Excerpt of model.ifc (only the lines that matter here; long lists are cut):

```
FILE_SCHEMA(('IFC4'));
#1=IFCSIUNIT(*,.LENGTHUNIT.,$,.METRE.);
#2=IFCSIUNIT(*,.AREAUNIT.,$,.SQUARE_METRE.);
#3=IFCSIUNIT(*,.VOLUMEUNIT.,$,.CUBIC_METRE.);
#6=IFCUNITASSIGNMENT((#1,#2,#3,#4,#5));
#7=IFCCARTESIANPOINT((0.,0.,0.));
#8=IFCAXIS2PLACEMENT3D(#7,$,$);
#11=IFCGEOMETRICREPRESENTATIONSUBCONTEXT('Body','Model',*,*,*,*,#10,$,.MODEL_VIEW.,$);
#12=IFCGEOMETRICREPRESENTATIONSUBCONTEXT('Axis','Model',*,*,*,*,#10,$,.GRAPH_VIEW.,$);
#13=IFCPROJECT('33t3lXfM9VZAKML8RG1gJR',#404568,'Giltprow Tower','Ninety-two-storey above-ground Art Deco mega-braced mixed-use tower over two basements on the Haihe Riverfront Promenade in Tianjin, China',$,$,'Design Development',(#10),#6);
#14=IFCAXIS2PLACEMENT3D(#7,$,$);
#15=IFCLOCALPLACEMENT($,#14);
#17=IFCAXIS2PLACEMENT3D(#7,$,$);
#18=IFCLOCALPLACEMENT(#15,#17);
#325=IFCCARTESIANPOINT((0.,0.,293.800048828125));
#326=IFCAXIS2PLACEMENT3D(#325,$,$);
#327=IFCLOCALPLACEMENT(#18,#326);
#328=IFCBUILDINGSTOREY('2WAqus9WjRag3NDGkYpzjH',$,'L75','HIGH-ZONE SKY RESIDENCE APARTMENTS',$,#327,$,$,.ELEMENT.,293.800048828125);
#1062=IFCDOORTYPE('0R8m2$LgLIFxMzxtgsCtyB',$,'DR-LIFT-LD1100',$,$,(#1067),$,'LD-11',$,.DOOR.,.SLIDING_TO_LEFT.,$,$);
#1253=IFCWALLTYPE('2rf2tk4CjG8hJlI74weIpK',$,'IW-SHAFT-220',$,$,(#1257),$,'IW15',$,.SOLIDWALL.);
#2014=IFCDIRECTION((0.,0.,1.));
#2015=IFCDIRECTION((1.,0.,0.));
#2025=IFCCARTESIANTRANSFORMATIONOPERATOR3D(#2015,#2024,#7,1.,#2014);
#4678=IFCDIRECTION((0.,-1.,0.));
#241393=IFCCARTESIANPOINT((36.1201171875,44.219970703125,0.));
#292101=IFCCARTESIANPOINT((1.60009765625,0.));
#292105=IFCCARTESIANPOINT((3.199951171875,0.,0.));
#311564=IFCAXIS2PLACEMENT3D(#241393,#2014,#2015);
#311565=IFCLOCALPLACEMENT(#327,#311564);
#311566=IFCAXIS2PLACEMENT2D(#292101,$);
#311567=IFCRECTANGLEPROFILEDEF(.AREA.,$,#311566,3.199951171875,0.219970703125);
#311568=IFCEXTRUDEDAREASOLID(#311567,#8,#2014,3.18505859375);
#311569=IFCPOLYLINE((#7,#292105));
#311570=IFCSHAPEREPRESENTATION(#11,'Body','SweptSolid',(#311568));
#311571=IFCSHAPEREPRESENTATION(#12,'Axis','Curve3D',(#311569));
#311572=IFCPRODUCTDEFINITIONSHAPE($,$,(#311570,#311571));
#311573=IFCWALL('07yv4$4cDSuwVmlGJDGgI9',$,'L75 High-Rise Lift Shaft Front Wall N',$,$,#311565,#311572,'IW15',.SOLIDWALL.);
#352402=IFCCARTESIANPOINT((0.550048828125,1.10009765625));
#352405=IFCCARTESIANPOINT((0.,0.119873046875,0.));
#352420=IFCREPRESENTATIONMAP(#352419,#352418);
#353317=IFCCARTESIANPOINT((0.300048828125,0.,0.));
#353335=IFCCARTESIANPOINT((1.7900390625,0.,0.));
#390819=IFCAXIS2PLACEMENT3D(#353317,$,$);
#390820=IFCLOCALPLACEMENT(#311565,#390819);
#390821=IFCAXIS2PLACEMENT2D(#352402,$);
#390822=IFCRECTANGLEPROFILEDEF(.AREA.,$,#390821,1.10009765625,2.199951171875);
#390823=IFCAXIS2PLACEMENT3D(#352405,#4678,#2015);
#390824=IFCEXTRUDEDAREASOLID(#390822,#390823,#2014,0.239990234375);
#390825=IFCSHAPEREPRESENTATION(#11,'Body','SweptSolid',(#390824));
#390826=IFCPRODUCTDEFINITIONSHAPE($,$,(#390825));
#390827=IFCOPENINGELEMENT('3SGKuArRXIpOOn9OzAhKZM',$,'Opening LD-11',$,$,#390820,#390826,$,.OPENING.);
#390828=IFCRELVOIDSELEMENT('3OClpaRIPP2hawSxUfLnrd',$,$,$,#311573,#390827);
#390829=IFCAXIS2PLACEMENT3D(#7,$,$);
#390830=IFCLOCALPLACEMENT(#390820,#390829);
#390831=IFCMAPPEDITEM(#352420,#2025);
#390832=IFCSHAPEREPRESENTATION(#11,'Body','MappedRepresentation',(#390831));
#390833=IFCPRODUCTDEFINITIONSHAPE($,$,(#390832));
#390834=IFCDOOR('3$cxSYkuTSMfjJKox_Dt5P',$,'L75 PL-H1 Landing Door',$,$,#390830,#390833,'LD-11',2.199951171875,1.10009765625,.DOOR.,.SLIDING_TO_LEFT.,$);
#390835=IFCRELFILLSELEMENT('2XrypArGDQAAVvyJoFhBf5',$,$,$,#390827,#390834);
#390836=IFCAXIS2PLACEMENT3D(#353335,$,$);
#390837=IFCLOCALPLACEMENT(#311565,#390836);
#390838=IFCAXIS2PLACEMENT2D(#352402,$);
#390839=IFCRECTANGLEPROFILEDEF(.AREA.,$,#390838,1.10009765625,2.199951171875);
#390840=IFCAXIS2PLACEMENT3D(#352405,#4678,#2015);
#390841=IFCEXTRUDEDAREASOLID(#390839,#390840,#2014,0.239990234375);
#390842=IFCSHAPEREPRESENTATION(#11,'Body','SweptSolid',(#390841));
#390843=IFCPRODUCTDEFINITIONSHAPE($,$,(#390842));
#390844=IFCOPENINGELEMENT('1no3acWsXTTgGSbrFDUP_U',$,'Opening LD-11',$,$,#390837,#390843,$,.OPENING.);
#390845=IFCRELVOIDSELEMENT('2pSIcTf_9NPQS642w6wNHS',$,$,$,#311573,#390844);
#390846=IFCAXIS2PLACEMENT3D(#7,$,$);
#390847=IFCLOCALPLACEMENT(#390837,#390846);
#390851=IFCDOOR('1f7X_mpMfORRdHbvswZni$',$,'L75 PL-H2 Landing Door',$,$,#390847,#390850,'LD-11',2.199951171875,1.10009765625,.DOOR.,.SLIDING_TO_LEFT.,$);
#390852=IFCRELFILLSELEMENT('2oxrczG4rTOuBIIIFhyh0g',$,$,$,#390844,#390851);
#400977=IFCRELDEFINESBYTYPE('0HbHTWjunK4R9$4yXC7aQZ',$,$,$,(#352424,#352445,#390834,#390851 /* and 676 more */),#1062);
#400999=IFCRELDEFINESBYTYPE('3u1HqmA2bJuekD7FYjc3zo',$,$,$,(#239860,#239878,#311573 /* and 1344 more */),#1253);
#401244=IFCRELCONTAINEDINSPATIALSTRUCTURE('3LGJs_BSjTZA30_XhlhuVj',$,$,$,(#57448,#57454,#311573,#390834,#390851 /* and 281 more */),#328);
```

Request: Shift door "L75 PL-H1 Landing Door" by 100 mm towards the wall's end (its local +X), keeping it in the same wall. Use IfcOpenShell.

```python
import ifcopenshell
import ifcopenshell.api.geometry
import ifcopenshell.util.placement
import ifcopenshell.util.unit

model = ifcopenshell.open("model.ifc")
unit_scale = ifcopenshell.util.unit.calculate_unit_scale(model)

door = model.by_guid("3$cxSYkuTSMfjJKox_Dt5P")
opening = door.FillsVoids[0].RelatingOpeningElement
wall = opening.VoidsElements[0].RelatingBuildingElement

wall_matrix = ifcopenshell.util.placement.get_local_placement(wall.ObjectPlacement)
shift = wall_matrix[:3, 0] * 0.1 / unit_scale
before = ifcopenshell.util.placement.get_local_placement(door.ObjectPlacement)[:3, 3].copy()

# The door is placed relative to its opening, so it follows when the opening moves.
matrix = ifcopenshell.util.placement.get_local_placement(opening.ObjectPlacement)
matrix[:3, 3] += shift
ifcopenshell.api.geometry.edit_object_placement(
    model, product=opening, matrix=matrix, is_si=False, should_transform_children=True
)

after = ifcopenshell.util.placement.get_local_placement(door.ObjectPlacement)[:3, 3]
print("door moved by", (after - before).round(3) + 0.0)

model.write("model_rev.ifc")
```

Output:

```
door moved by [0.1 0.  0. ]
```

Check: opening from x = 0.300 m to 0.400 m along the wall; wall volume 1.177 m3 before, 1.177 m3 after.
